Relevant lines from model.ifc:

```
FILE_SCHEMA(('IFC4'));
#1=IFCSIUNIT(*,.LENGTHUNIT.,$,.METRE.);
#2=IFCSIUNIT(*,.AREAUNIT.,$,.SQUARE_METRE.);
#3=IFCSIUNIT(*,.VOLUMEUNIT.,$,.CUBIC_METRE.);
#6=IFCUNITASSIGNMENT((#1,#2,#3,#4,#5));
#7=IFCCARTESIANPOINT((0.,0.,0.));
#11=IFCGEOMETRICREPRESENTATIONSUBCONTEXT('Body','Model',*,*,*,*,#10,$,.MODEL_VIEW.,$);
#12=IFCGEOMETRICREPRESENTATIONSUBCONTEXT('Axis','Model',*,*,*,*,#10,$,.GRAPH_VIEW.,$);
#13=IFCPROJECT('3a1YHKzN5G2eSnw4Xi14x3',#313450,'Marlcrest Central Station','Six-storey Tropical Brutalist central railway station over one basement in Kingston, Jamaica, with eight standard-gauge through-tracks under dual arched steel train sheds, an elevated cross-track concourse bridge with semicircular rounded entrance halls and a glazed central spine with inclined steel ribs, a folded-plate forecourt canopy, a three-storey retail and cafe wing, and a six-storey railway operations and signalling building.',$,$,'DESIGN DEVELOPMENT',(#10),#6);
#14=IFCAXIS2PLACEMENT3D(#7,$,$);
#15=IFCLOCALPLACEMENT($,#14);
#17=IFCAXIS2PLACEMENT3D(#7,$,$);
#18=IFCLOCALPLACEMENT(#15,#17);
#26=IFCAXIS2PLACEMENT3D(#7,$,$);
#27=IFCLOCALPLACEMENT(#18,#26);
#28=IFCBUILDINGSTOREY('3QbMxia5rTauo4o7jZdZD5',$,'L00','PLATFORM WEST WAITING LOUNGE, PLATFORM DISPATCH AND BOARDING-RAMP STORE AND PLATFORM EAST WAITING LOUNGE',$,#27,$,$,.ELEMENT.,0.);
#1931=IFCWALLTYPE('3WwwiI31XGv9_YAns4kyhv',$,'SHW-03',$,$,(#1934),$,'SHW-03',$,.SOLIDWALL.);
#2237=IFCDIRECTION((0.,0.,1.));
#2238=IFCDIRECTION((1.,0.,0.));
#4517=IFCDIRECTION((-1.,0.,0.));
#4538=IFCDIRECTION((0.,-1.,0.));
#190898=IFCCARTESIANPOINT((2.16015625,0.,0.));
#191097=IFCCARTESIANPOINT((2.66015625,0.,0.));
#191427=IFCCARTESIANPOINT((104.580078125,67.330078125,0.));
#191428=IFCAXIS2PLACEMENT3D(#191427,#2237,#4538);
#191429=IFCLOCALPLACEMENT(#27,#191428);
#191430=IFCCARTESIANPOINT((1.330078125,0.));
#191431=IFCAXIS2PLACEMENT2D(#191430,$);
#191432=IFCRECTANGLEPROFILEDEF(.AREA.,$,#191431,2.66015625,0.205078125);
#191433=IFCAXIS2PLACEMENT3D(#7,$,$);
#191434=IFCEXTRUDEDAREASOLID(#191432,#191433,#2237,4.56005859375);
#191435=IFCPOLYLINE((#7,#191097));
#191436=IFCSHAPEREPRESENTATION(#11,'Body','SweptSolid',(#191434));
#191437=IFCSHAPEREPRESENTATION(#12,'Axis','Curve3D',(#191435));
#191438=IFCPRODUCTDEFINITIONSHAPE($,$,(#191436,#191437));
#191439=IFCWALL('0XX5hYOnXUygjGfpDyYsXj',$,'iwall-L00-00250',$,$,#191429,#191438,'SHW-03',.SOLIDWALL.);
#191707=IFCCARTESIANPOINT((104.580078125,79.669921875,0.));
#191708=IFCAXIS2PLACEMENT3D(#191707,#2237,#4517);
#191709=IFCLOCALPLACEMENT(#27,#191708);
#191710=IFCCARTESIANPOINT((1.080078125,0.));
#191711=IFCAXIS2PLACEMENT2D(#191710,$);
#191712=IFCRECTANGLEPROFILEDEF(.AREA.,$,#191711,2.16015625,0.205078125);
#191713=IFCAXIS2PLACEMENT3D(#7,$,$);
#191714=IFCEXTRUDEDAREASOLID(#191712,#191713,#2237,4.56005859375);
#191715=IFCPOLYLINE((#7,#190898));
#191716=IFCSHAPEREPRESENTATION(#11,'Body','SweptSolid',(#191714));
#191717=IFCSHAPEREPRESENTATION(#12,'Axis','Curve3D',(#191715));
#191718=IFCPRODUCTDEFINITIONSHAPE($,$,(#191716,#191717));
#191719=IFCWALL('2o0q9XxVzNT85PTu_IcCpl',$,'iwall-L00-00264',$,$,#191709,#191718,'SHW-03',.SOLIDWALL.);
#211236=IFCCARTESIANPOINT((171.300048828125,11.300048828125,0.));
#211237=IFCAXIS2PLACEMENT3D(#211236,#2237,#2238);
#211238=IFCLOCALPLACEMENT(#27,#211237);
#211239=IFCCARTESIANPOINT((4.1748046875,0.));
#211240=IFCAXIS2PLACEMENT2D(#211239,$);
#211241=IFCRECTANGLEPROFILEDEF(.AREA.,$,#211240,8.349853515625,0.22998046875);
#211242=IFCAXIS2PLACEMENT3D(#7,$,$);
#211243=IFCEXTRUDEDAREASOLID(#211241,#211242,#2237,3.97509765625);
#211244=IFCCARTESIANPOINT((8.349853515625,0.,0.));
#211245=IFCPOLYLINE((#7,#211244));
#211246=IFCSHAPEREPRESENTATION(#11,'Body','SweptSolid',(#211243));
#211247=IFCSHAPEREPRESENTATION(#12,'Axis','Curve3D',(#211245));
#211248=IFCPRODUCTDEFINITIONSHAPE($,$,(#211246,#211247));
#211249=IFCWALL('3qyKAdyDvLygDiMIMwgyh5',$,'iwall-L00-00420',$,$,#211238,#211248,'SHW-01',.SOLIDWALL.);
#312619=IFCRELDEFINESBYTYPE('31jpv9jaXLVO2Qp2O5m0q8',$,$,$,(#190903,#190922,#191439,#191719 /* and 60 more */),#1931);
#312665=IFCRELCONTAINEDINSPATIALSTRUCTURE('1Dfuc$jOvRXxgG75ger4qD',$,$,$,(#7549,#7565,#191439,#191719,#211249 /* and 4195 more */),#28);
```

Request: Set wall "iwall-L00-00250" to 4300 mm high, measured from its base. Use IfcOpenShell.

```python
import ifcopenshell
import ifcopenshell.geom
import ifcopenshell.util.representation
import ifcopenshell.util.shape
import ifcopenshell.util.unit

model = ifcopenshell.open("model.ifc")
unit_scale = ifcopenshell.util.unit.calculate_unit_scale(model)
settings = ifcopenshell.geom.settings()


def volume(element):
    """Net volume in cubic metres, openings subtracted."""
    shape = ifcopenshell.geom.create_shape(settings, element)
    return ifcopenshell.util.shape.get_volume(shape.geometry)


wall = model.by_guid("0XX5hYOnXUygjGfpDyYsXj")
before = volume(wall)

body = ifcopenshell.util.representation.get_representation(wall, "Model", "Body")
solid = body.Items[0]
old_height = solid.Depth
solid.Depth = 4.3 / unit_scale
after = volume(wall)

print(f"height {old_height:g} -> {solid.Depth:g}, volume {before:.3f} -> {after:.3f} m3")

model.write("model_updated.ifc")
```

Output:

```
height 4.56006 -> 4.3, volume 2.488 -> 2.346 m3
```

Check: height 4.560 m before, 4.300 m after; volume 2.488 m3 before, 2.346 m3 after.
